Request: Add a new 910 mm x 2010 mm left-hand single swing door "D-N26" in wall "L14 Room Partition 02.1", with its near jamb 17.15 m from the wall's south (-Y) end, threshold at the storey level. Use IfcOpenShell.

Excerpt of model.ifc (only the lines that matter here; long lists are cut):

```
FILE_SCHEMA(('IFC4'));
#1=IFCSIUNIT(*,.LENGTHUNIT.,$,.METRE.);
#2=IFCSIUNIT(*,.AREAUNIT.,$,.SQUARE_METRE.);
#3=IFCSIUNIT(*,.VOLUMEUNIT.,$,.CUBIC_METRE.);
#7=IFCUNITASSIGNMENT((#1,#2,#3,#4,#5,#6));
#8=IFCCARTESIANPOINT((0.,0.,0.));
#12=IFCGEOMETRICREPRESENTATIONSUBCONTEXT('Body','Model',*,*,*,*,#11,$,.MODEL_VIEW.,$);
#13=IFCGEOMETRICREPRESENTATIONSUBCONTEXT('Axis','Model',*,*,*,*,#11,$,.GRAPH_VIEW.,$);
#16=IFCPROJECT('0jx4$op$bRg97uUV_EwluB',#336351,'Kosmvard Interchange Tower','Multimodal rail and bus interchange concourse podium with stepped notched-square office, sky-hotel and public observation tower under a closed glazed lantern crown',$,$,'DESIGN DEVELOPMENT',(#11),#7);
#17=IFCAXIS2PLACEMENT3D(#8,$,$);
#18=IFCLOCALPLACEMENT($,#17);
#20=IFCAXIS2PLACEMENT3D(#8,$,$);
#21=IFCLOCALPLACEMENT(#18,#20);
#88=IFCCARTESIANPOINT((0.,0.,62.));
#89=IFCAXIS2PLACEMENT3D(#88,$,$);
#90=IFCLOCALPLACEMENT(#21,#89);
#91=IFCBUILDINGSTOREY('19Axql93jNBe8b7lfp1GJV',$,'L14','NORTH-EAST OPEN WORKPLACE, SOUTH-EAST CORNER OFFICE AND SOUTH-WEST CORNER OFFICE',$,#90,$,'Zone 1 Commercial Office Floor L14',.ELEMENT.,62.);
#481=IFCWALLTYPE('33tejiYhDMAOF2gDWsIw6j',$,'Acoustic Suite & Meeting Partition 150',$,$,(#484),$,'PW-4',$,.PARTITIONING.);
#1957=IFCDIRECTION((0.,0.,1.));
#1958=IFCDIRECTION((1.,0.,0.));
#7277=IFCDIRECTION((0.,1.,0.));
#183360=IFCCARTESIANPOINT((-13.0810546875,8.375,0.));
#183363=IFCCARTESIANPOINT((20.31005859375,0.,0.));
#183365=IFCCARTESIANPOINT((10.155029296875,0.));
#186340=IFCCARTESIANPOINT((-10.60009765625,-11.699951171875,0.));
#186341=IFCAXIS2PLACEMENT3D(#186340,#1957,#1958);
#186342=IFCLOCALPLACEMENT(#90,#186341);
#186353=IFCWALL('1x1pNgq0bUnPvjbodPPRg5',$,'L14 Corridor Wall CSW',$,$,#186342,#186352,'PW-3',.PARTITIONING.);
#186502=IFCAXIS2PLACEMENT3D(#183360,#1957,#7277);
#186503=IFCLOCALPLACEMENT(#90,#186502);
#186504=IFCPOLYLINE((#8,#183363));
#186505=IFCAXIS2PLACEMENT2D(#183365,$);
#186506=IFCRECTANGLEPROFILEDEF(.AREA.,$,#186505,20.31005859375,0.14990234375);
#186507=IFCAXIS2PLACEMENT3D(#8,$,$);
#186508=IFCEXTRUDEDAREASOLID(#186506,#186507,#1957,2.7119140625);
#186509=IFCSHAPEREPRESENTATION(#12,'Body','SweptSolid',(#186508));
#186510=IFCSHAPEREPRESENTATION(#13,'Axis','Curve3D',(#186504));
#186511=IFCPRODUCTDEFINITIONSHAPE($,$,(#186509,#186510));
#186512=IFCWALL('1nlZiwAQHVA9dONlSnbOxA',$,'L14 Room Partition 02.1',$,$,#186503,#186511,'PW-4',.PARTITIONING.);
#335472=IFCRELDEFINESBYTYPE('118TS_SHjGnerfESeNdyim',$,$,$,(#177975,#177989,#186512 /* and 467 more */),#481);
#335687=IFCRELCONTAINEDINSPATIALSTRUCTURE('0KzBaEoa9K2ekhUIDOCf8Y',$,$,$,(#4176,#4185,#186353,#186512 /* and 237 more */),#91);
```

```python
import numpy as np
import ifcopenshell
import ifcopenshell.api.feature
import ifcopenshell.api.geometry
import ifcopenshell.api.root
import ifcopenshell.api.spatial
import ifcopenshell.geom
import ifcopenshell.util.element
import ifcopenshell.util.placement
import ifcopenshell.util.representation
import ifcopenshell.util.shape
import ifcopenshell.util.unit

model = ifcopenshell.open("model.ifc")
unit_scale = ifcopenshell.util.unit.calculate_unit_scale(model)
settings = ifcopenshell.geom.settings()


def volume(element):
    """Net volume in cubic metres, openings subtracted."""
    shape = ifcopenshell.geom.create_shape(settings, element)
    return ifcopenshell.util.shape.get_volume(shape.geometry)


wall = model.by_id(186512)
storey = ifcopenshell.util.element.get_container(wall, ifc_class="IfcBuildingStorey")
context = ifcopenshell.util.representation.get_context(model, "Model", "Body", "MODEL_VIEW")
before = volume(wall)

width, height, from_end, sill = 0.91, 2.01, 17.15, 0.0  # metres

# The wall runs along its own X axis, and the end named is its -X end.
wall_shape = ifcopenshell.geom.create_shape(settings, wall)
x, y, z = ifcopenshell.util.shape.get_vertices(wall_shape.geometry).T
start = x.min() + from_end
face, thickness = float(y.min()), float(y.max() - y.min())
wall_matrix = ifcopenshell.util.placement.get_local_placement(wall.ObjectPlacement)
level = ifcopenshell.util.placement.get_local_placement(storey.ObjectPlacement)[2, 3]


def in_wall(x, y):
    """Placement at x, y metres in the wall's axes, at sill height."""
    matrix = wall_matrix.copy()
    matrix[:, 3] = wall_matrix @ np.array([x / unit_scale, y / unit_scale, 0.0, 1.0])
    matrix[2, 3] = level + sill / unit_scale
    return matrix


# Opening: a box that overshoots both wall faces by 50 mm.
opening = ifcopenshell.api.root.create_entity(model, ifc_class="IfcOpeningElement", predefined_type="OPENING")
box = ifcopenshell.api.geometry.add_wall_representation(
    model, context=context, length=width, height=height, thickness=thickness + 0.1
)
ifcopenshell.api.geometry.assign_representation(model, product=opening, representation=box)
ifcopenshell.api.geometry.edit_object_placement(model, product=opening, matrix=in_wall(start, face - 0.05), is_si=False)
ifcopenshell.api.feature.add_feature(model, feature=opening, element=wall)

door = ifcopenshell.api.root.create_entity(model, ifc_class="IfcDoor", name="D-N26", predefined_type="DOOR")
door.OverallWidth, door.OverallHeight = width / unit_scale, height / unit_scale
door.OperationType = "SINGLE_SWING_LEFT"
body = ifcopenshell.api.geometry.add_door_representation(
    model,
    context=context,
    overall_width=door.OverallWidth,
    overall_height=door.OverallHeight,
    operation_type="SINGLE_SWING_LEFT",
    lining_properties={"LiningDepth": thickness / unit_scale, "ThresholdDepth": thickness / unit_scale},
)
ifcopenshell.api.geometry.assign_representation(model, product=door, representation=body)
ifcopenshell.api.spatial.assign_container(model, products=[door], relating_structure=storey)
ifcopenshell.api.feature.add_filling(model, opening=opening, element=door)

# The lining spans the wall, so the door starts at the wall face.
ifcopenshell.api.geometry.edit_object_placement(model, product=door, matrix=in_wall(start, face), is_si=False)

after = volume(wall)

print(f"wall volume {before:.3f} -> {after:.3f} m3")

model.write("model_v2.ifc")
```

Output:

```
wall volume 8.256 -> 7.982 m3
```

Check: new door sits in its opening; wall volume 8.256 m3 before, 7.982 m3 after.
